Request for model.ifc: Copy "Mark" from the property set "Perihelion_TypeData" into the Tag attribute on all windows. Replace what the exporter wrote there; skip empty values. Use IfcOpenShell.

First a look at what the model holds.

```python
import ifcopenshell
import ifcopenshell.util.element

model = ifcopenshell.open("model.ifc")
print(model.schema)
windows = model.by_type("IfcWindow")
print(len(windows), "windows")
for e in windows[:8]:
    source = ifcopenshell.util.element.get_pset(e, "Perihelion_TypeData", "Mark")
    target = e.Tag
    print(e.id(), repr(source), repr(target), sep=" | ")
```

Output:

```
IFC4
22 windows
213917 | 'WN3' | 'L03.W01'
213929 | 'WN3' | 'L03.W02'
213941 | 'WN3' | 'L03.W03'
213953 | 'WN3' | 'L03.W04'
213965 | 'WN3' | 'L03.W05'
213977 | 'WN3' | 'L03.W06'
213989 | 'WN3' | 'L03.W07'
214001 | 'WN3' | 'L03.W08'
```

```python
import ifcopenshell
import ifcopenshell.util.element

model = ifcopenshell.open("model.ifc")

count = 0
for e in model.by_type("IfcWindow"):
    value = ifcopenshell.util.element.get_pset(e, "Perihelion_TypeData", "Mark")
    current = e.Tag
    if not value or not value.strip() or current == value:
        continue
    e.Tag = value
    count += 1

print(count, "windows updated")

model.write("model_edited.ifc")
```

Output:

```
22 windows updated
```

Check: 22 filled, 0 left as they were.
